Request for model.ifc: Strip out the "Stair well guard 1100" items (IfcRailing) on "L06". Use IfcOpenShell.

First a look at what the model holds.

```python
import ifcopenshell
import ifcopenshell.util.element

model = ifcopenshell.open("model.ifc")
print(model.schema)
storey = next(s for s in model.by_type("IfcBuildingStorey") if s.Name == "L06")
railings = [e for e in ifcopenshell.util.element.get_decomposition(storey) if e.is_a("IfcRailing")]
seen = {}
for e in railings:
    element_type = ifcopenshell.util.element.get_type(e)
    name = element_type.Name if element_type not in (None, e) else None
    seen[name] = seen.get(name, 0) + 1
for name, count in sorted(seen.items(), key=str):
    print(count, "x", name)
```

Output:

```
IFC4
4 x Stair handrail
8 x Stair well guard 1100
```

```python
import ifcopenshell
import ifcopenshell.api.root
import ifcopenshell.util.element

model = ifcopenshell.open("model.ifc")

storey = next(s for s in model.by_type("IfcBuildingStorey") if s.Name == "L06")
railings = [e for e in ifcopenshell.util.element.get_decomposition(storey) if e.is_a("IfcRailing")]
targets = [e for e in railings if (t := ifcopenshell.util.element.get_type(e)) not in (None, e) and t.Name == "Stair well guard 1100"]

for e in targets:
    ifcopenshell.api.root.remove_product(model, product=e)
print(len(targets), "removed")

model.write("model_edited.ifc")
```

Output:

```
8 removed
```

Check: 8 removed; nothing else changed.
